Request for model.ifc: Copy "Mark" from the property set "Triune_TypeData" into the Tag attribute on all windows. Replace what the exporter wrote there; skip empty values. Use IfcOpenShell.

First a look at what the model holds.

```python
import ifcopenshell
import ifcopenshell.util.element

model = ifcopenshell.open("model.ifc")
print(model.schema)
windows = model.by_type("IfcWindow")
print(len(windows), "windows")
for e in windows[:8]:
    source = ifcopenshell.util.element.get_pset(e, "Triune_TypeData", "Mark")
    target = e.Tag
    print(e.id(), repr(source), repr(target), sep=" | ")
```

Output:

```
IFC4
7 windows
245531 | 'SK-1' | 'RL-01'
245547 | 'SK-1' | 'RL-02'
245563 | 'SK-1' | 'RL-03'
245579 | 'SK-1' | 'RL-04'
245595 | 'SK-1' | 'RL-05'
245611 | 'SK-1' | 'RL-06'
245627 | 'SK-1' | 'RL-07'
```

```python
import ifcopenshell
import ifcopenshell.util.element

model = ifcopenshell.open("model.ifc")

count = 0
for e in model.by_type("IfcWindow"):
    value = ifcopenshell.util.element.get_pset(e, "Triune_TypeData", "Mark")
    current = e.Tag
    if not value or not value.strip() or current == value:
        continue
    e.Tag = value
    count += 1

print(count, "windows updated")

model.write("model-out.ifc")
```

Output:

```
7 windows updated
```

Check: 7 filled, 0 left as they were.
